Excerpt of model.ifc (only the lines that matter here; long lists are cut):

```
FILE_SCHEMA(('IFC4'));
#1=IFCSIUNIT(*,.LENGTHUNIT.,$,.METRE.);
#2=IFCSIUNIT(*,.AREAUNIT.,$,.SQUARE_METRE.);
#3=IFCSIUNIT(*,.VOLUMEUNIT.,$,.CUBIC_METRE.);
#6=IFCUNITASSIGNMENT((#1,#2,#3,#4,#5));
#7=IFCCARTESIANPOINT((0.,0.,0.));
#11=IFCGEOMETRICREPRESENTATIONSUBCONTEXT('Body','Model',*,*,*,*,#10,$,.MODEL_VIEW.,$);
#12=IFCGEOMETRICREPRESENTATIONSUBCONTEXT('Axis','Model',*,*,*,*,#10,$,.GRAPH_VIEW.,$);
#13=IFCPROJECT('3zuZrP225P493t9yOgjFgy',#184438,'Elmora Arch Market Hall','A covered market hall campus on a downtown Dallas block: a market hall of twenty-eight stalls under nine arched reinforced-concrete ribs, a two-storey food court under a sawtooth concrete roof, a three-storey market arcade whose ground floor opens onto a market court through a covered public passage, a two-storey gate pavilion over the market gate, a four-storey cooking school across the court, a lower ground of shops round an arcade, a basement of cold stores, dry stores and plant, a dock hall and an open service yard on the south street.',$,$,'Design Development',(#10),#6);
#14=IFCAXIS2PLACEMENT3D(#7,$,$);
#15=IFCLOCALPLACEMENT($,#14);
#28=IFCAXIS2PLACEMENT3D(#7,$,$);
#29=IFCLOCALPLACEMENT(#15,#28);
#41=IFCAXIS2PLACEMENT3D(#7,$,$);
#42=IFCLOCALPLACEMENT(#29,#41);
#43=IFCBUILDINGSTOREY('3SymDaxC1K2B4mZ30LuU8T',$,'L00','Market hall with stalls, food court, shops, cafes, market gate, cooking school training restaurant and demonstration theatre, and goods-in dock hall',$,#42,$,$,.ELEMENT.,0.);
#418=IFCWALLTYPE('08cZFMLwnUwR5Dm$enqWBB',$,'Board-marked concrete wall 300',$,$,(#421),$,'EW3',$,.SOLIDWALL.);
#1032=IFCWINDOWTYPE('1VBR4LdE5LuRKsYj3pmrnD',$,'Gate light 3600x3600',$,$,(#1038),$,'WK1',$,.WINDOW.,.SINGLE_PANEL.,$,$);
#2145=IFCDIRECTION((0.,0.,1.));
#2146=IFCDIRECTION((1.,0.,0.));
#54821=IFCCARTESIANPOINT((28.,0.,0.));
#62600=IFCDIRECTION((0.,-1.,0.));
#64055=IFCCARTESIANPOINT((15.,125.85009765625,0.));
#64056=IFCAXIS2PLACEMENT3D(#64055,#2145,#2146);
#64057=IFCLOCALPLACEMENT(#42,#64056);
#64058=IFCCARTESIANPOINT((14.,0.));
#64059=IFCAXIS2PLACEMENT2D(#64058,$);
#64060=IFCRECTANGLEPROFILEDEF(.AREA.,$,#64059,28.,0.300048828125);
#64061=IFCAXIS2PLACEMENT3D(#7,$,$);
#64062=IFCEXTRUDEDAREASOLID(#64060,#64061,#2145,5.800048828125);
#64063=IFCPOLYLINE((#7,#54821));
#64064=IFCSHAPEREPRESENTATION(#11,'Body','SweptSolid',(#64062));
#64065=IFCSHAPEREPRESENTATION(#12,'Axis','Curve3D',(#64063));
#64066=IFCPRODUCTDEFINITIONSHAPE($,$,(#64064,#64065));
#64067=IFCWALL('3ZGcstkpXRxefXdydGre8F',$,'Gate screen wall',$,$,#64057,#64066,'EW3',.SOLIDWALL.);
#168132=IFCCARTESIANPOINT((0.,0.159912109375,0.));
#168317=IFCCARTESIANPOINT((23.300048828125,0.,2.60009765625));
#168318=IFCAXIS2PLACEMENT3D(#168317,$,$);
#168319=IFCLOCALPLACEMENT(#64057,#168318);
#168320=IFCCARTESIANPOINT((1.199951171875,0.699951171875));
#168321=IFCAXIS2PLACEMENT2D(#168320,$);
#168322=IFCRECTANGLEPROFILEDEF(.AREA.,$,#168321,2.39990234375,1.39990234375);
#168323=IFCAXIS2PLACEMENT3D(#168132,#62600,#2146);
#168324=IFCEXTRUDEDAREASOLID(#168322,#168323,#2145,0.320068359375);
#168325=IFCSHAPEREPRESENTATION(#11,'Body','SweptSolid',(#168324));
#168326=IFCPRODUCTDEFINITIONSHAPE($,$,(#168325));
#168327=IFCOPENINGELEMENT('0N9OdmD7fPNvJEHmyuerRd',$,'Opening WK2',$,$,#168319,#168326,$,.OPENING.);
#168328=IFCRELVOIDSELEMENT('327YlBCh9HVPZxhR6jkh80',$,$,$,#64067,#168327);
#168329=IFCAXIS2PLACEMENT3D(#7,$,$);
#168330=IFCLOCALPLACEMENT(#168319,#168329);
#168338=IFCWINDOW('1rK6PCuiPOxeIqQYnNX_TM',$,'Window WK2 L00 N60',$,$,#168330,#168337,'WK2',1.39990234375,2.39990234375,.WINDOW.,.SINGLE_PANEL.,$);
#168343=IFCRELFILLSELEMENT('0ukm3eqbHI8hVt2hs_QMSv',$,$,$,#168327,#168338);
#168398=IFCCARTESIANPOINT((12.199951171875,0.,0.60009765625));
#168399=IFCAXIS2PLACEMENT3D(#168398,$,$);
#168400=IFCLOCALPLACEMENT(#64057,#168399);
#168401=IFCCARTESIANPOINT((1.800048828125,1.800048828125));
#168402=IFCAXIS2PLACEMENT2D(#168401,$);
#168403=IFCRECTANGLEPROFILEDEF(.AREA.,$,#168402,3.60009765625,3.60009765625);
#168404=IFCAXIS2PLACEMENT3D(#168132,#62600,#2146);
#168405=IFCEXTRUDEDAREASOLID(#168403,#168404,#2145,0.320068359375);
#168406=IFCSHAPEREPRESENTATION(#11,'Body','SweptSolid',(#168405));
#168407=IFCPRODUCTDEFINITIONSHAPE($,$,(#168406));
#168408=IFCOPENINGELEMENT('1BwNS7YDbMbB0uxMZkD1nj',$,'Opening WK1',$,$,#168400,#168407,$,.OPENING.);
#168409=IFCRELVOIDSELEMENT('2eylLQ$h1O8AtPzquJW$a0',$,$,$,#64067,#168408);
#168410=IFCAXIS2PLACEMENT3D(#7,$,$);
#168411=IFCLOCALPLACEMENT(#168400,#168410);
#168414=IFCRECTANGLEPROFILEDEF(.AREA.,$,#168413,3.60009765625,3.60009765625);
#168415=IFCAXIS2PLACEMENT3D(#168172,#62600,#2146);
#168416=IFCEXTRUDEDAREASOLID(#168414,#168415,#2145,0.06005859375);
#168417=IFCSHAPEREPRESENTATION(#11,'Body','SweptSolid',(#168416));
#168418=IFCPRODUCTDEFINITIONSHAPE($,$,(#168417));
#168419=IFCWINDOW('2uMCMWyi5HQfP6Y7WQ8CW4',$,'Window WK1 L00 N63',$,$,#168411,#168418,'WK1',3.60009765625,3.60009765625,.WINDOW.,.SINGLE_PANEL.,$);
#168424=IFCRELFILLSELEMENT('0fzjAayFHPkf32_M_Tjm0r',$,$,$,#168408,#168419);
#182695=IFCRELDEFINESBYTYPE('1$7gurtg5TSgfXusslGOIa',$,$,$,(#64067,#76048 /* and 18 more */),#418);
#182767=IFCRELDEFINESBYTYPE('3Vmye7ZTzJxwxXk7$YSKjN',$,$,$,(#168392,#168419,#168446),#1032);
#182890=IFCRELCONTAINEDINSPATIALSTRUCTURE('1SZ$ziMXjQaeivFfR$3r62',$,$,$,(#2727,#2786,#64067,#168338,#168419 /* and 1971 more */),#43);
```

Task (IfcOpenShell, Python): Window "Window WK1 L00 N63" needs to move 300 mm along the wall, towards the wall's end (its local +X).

```python
import ifcopenshell
import ifcopenshell.api.geometry
import ifcopenshell.util.placement

model = ifcopenshell.open("model.ifc")

window = model.by_guid("2uMCMWyi5HQfP6Y7WQ8CW4")
opening = window.FillsVoids[0].RelatingOpeningElement
wall = opening.VoidsElements[0].RelatingBuildingElement

wall_matrix = ifcopenshell.util.placement.get_local_placement(wall.ObjectPlacement)
shift = wall_matrix[:3, 0] * 0.3
before = ifcopenshell.util.placement.get_local_placement(window.ObjectPlacement)[:3, 3].copy()

# The window is placed relative to its opening, so it follows when the opening moves.
matrix = ifcopenshell.util.placement.get_local_placement(opening.ObjectPlacement)
matrix[:3, 3] += shift
ifcopenshell.api.geometry.edit_object_placement(
    model, product=opening, matrix=matrix, is_si=False, should_transform_children=True
)

after = ifcopenshell.util.placement.get_local_placement(window.ObjectPlacement)[:3, 3]
print("window moved by", (after - before).round(3) + 0.0)

model.write("model_edited.ifc")
```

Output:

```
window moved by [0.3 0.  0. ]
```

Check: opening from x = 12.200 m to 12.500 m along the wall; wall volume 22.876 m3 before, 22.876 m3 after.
